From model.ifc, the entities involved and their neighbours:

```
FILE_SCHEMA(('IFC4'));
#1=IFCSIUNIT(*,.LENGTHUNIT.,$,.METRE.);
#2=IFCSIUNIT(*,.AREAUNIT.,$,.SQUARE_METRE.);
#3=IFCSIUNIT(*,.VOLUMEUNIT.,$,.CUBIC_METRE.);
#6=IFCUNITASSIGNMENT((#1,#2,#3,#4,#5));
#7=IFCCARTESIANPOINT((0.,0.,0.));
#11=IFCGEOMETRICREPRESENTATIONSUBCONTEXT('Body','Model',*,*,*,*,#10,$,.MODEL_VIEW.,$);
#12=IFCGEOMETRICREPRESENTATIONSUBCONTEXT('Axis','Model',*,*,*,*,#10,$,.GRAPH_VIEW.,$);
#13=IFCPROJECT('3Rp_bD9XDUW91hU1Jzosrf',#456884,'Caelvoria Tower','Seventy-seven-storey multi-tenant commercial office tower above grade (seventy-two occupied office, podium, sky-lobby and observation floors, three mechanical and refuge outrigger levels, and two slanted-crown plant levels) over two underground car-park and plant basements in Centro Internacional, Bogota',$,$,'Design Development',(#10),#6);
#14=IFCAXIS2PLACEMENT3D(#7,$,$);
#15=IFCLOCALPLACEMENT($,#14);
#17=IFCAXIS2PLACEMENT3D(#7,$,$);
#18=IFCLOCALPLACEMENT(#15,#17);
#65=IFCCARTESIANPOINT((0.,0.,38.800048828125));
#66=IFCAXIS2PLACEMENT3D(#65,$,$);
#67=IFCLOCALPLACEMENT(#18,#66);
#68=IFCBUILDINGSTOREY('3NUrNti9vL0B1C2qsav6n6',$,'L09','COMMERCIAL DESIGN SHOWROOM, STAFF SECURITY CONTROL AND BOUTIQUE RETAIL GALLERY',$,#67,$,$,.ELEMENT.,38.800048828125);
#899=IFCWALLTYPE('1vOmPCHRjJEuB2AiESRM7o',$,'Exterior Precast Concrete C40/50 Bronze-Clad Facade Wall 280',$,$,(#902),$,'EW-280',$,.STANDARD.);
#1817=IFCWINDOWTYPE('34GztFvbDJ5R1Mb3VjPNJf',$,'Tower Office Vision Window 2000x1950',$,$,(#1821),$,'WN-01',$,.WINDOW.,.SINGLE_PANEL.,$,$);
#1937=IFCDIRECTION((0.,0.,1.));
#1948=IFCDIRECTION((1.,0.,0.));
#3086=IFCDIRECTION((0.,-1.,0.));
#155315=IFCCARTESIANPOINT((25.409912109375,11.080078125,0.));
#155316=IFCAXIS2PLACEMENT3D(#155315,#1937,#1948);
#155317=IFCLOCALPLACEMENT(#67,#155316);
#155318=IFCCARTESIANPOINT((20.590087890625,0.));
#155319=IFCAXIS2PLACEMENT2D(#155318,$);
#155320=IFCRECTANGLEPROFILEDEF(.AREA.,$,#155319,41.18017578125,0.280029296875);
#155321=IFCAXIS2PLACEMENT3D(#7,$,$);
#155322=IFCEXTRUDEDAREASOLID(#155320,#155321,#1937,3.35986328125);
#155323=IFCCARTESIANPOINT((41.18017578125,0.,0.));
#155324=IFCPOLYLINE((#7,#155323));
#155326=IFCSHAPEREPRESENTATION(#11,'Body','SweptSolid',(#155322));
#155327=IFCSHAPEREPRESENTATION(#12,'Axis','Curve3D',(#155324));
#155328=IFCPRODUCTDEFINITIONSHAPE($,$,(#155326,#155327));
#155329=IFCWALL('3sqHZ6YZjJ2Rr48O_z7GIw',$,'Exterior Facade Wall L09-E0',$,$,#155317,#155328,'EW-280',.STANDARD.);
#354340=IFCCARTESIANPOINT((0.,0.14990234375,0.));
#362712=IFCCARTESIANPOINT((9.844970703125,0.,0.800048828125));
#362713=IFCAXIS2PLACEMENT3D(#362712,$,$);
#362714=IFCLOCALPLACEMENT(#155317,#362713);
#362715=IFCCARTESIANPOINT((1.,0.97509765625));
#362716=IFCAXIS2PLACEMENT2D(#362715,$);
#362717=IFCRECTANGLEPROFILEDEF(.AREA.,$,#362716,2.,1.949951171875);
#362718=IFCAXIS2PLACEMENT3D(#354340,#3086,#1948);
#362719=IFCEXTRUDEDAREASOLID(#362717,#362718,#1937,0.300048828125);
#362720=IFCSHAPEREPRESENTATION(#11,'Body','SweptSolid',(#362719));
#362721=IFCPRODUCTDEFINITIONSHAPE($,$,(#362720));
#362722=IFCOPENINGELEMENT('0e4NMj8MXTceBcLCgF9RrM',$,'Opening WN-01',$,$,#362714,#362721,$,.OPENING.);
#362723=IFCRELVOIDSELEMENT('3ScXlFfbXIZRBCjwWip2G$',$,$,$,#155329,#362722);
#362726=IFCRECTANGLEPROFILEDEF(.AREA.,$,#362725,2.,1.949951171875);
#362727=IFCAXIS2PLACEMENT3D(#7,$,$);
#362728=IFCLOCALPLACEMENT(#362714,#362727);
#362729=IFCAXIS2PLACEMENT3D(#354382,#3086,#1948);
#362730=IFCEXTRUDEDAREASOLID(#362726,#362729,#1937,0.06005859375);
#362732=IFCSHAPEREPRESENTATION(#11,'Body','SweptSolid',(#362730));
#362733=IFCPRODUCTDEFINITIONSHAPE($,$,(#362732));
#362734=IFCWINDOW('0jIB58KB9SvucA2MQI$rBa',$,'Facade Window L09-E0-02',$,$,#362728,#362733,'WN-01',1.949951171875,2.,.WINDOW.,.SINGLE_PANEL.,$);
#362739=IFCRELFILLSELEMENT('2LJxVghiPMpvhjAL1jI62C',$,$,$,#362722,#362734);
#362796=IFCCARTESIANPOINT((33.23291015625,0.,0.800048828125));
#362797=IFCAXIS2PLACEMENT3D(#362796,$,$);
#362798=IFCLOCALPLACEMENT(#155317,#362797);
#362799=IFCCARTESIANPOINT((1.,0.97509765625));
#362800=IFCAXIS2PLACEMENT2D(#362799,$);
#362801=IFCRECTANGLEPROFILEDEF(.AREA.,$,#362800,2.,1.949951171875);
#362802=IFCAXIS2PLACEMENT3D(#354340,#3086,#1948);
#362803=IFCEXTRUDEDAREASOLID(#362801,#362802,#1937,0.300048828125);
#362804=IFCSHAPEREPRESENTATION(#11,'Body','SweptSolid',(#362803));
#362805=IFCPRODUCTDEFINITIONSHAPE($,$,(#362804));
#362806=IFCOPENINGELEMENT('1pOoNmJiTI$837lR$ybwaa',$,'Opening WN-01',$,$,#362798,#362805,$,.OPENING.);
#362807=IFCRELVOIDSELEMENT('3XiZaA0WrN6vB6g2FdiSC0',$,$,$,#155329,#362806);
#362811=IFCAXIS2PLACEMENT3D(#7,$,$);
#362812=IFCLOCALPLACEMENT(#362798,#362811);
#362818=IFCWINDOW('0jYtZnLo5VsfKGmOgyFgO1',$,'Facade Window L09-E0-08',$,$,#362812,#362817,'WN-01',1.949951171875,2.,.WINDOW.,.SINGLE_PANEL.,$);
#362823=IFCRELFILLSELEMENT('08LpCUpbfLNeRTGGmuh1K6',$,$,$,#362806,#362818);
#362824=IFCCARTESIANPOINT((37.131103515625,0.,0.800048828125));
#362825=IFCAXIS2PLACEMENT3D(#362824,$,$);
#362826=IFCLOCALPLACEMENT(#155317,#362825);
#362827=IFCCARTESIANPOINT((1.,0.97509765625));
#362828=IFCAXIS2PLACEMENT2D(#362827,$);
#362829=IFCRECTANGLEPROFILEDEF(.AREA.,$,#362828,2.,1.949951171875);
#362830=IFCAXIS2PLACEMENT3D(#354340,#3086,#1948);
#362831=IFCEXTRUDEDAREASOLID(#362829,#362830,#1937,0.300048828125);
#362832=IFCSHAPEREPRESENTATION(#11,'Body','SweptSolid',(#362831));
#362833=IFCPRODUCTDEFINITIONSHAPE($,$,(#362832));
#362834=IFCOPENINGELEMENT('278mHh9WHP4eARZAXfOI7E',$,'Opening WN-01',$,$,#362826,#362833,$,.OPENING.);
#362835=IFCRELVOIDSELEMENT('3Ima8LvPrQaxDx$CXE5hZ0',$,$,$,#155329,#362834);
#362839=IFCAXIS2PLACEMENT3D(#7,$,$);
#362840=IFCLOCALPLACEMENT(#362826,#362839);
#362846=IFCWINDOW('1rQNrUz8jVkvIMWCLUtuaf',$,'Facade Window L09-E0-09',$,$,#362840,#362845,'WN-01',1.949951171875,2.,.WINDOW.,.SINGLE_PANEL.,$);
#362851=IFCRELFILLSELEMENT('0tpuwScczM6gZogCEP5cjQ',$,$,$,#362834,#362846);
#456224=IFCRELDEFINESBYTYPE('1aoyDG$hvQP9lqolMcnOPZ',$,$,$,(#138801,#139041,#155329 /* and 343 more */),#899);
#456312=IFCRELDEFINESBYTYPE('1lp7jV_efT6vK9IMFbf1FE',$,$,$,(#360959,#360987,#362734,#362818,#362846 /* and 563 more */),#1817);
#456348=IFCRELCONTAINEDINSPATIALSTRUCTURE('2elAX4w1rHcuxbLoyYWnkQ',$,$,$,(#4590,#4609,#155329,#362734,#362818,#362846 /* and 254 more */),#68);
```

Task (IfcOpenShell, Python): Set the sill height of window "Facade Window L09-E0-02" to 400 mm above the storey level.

```python
import numpy as np
import ifcopenshell
import ifcopenshell.api.geometry
import ifcopenshell.geom
import ifcopenshell.util.element
import ifcopenshell.util.placement
import ifcopenshell.util.shape
import ifcopenshell.util.unit

model = ifcopenshell.open("model.ifc")
unit_scale = ifcopenshell.util.unit.calculate_unit_scale(model)

window = model.by_id(362734)
opening = window.FillsVoids[0].RelatingOpeningElement
storey = ifcopenshell.util.element.get_container(window, ifc_class="IfcBuildingStorey")
level = ifcopenshell.util.placement.get_local_placement(storey.ObjectPlacement)[2, 3]

# The opening's origin need not be at the sill, so measure its lowest point.
shape = ifcopenshell.geom.create_shape(ifcopenshell.geom.settings(), opening)
bottom = ifcopenshell.util.shape.get_shape_bottom_elevation(shape, shape.geometry) / unit_scale
dz = level + 0.4 - bottom

shift = np.array([0.0, 0.0, dz])
# The window is placed relative to its opening, so it follows when the opening moves.
matrix = ifcopenshell.util.placement.get_local_placement(opening.ObjectPlacement)
matrix[:3, 3] += shift
ifcopenshell.api.geometry.edit_object_placement(
    model, product=opening, matrix=matrix, is_si=False, should_transform_children=True
)

print(f"moved by {dz * unit_scale:+.3f} m")

model.write("model_updated.ifc")
```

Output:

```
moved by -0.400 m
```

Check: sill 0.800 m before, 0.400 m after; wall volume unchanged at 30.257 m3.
